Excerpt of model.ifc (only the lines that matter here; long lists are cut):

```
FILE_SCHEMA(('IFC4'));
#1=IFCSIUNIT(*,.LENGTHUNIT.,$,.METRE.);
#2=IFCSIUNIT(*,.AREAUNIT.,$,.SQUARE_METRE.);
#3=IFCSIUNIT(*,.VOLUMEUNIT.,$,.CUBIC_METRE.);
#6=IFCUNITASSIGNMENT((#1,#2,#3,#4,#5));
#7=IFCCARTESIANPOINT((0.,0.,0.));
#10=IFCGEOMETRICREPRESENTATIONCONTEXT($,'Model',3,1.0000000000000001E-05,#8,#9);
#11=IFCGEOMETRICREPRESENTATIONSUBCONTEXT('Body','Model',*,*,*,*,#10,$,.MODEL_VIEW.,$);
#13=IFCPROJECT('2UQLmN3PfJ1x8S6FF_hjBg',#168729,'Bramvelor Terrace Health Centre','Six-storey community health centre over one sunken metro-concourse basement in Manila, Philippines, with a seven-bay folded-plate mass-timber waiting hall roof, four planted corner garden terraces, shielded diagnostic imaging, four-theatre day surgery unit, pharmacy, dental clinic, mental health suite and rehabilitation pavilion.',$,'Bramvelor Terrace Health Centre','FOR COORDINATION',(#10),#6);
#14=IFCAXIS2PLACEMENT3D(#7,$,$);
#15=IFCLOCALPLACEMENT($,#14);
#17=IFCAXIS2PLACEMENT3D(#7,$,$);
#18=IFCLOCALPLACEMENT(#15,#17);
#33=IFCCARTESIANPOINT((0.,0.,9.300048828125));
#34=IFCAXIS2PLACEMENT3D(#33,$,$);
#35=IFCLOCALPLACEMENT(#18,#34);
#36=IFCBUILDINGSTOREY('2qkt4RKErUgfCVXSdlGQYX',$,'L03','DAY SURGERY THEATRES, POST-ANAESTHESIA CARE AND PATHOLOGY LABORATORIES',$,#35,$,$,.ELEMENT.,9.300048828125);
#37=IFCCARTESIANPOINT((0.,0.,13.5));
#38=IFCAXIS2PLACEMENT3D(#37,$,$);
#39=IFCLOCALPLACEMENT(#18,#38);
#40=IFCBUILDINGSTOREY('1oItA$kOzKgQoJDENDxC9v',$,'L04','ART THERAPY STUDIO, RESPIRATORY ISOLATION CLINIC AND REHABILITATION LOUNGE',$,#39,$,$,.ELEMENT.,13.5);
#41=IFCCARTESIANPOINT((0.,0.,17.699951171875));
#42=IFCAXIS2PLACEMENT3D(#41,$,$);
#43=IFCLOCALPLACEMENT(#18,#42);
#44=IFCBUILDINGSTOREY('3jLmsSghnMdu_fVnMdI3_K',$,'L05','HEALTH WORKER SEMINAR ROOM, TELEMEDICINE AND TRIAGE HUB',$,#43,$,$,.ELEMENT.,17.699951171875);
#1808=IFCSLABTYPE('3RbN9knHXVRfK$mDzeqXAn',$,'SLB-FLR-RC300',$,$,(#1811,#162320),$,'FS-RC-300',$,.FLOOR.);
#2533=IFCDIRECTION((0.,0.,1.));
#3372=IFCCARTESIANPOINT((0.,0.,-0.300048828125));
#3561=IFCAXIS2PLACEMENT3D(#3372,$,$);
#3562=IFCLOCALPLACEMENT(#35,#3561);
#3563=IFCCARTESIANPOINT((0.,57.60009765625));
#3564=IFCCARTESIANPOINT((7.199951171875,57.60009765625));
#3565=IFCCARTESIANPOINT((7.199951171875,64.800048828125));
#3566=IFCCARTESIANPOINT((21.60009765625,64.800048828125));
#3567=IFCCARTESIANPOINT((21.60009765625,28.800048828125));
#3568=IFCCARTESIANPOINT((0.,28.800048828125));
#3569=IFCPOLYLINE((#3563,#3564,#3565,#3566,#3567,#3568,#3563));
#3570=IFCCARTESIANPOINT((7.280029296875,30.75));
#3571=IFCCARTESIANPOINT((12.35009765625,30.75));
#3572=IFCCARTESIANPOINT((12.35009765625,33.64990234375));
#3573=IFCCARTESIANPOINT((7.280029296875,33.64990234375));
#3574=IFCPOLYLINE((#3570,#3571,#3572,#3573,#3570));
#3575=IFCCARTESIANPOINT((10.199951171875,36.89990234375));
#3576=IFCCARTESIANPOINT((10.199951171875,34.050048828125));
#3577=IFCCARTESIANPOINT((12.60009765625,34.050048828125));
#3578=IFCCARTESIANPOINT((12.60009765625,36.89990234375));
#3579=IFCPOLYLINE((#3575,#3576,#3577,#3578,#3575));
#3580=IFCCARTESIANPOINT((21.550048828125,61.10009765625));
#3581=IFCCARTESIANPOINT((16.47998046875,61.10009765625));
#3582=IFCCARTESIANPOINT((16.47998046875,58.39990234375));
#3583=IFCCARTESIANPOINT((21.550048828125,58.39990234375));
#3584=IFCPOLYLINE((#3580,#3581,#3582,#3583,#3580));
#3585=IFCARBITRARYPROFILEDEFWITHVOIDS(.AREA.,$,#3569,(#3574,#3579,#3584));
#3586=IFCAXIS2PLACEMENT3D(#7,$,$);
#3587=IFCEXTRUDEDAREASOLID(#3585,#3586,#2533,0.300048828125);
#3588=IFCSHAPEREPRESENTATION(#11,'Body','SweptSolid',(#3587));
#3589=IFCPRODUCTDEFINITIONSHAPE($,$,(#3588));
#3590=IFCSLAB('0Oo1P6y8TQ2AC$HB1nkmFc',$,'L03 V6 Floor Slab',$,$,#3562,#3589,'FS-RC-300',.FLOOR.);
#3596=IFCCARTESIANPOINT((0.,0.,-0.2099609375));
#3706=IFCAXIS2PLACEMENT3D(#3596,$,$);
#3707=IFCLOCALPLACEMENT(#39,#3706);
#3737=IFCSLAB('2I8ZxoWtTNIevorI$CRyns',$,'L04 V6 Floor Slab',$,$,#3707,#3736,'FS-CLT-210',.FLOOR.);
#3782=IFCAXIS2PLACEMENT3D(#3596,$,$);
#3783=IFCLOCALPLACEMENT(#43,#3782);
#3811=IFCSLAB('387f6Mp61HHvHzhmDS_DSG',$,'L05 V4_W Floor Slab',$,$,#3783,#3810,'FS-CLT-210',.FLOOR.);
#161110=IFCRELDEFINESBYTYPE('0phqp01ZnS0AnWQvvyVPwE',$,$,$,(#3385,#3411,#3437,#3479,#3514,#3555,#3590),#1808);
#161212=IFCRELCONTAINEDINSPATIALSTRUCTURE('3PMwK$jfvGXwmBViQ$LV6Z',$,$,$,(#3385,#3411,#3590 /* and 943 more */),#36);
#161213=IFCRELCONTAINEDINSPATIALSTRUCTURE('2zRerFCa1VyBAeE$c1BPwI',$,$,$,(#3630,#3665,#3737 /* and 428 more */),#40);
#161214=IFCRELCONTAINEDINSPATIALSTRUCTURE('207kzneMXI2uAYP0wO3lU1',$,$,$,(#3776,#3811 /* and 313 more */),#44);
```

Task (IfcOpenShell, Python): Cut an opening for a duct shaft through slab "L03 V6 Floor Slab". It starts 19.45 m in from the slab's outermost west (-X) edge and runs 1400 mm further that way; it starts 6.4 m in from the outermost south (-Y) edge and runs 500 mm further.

```python
import numpy as np
import ifcopenshell
import ifcopenshell.api.feature
import ifcopenshell.api.geometry
import ifcopenshell.api.root
import ifcopenshell.geom
import ifcopenshell.util.placement
import ifcopenshell.util.representation
import ifcopenshell.util.shape
import ifcopenshell.util.unit

model = ifcopenshell.open("model.ifc")
unit_scale = ifcopenshell.util.unit.calculate_unit_scale(model)
settings = ifcopenshell.geom.settings()


def volume(element):
    """Net volume in cubic metres, openings subtracted."""
    shape = ifcopenshell.geom.create_shape(settings, element)
    return ifcopenshell.util.shape.get_volume(shape.geometry)


slab = model.by_guid("0Oo1P6y8TQ2AC$HB1nkmFc")
before = volume(slab)

# Extent in the slab's own axes, in metres. The edges named are its -X and -Y sides.
slab_shape = ifcopenshell.geom.create_shape(settings, slab)
vertices = ifcopenshell.util.shape.get_vertices(slab_shape.geometry)
x_min, y_min, bottom = vertices.min(axis=0)
top = vertices[:, 2].max()

opening = ifcopenshell.api.root.create_entity(model, ifc_class="IfcOpeningElement", name="Duct shaft opening", predefined_type="OPENING")
context = ifcopenshell.util.representation.get_context(model, "Model", "Body", "MODEL_VIEW")
width, depth = 1.4, 0.5
outline = [(0.0, 0.0), (width, 0.0), (width, depth), (0.0, depth), (0.0, 0.0)]
# Overshoot both faces by 50 mm so the cut is clean.
shape = ifcopenshell.api.geometry.add_slab_representation(
    model, context=context, depth=top - bottom + 0.1, polyline=outline
)
ifcopenshell.api.geometry.assign_representation(model, product=opening, representation=shape)

matrix = ifcopenshell.util.placement.get_local_placement(slab.ObjectPlacement)
matrix[:, 3] = matrix @ np.append(np.array([x_min + 19.45, y_min + 6.4, bottom - 0.05]) / unit_scale, 1.0)
ifcopenshell.api.geometry.edit_object_placement(model, product=opening, matrix=matrix, is_si=False)
ifcopenshell.api.feature.add_feature(model, feature=opening, element=slab)

after = volume(slab)

print(f"slab volume {before:.3f} -> {after:.3f} m3")

model.write("model_edited.ifc")
```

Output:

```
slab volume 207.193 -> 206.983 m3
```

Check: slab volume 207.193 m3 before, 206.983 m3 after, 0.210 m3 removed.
